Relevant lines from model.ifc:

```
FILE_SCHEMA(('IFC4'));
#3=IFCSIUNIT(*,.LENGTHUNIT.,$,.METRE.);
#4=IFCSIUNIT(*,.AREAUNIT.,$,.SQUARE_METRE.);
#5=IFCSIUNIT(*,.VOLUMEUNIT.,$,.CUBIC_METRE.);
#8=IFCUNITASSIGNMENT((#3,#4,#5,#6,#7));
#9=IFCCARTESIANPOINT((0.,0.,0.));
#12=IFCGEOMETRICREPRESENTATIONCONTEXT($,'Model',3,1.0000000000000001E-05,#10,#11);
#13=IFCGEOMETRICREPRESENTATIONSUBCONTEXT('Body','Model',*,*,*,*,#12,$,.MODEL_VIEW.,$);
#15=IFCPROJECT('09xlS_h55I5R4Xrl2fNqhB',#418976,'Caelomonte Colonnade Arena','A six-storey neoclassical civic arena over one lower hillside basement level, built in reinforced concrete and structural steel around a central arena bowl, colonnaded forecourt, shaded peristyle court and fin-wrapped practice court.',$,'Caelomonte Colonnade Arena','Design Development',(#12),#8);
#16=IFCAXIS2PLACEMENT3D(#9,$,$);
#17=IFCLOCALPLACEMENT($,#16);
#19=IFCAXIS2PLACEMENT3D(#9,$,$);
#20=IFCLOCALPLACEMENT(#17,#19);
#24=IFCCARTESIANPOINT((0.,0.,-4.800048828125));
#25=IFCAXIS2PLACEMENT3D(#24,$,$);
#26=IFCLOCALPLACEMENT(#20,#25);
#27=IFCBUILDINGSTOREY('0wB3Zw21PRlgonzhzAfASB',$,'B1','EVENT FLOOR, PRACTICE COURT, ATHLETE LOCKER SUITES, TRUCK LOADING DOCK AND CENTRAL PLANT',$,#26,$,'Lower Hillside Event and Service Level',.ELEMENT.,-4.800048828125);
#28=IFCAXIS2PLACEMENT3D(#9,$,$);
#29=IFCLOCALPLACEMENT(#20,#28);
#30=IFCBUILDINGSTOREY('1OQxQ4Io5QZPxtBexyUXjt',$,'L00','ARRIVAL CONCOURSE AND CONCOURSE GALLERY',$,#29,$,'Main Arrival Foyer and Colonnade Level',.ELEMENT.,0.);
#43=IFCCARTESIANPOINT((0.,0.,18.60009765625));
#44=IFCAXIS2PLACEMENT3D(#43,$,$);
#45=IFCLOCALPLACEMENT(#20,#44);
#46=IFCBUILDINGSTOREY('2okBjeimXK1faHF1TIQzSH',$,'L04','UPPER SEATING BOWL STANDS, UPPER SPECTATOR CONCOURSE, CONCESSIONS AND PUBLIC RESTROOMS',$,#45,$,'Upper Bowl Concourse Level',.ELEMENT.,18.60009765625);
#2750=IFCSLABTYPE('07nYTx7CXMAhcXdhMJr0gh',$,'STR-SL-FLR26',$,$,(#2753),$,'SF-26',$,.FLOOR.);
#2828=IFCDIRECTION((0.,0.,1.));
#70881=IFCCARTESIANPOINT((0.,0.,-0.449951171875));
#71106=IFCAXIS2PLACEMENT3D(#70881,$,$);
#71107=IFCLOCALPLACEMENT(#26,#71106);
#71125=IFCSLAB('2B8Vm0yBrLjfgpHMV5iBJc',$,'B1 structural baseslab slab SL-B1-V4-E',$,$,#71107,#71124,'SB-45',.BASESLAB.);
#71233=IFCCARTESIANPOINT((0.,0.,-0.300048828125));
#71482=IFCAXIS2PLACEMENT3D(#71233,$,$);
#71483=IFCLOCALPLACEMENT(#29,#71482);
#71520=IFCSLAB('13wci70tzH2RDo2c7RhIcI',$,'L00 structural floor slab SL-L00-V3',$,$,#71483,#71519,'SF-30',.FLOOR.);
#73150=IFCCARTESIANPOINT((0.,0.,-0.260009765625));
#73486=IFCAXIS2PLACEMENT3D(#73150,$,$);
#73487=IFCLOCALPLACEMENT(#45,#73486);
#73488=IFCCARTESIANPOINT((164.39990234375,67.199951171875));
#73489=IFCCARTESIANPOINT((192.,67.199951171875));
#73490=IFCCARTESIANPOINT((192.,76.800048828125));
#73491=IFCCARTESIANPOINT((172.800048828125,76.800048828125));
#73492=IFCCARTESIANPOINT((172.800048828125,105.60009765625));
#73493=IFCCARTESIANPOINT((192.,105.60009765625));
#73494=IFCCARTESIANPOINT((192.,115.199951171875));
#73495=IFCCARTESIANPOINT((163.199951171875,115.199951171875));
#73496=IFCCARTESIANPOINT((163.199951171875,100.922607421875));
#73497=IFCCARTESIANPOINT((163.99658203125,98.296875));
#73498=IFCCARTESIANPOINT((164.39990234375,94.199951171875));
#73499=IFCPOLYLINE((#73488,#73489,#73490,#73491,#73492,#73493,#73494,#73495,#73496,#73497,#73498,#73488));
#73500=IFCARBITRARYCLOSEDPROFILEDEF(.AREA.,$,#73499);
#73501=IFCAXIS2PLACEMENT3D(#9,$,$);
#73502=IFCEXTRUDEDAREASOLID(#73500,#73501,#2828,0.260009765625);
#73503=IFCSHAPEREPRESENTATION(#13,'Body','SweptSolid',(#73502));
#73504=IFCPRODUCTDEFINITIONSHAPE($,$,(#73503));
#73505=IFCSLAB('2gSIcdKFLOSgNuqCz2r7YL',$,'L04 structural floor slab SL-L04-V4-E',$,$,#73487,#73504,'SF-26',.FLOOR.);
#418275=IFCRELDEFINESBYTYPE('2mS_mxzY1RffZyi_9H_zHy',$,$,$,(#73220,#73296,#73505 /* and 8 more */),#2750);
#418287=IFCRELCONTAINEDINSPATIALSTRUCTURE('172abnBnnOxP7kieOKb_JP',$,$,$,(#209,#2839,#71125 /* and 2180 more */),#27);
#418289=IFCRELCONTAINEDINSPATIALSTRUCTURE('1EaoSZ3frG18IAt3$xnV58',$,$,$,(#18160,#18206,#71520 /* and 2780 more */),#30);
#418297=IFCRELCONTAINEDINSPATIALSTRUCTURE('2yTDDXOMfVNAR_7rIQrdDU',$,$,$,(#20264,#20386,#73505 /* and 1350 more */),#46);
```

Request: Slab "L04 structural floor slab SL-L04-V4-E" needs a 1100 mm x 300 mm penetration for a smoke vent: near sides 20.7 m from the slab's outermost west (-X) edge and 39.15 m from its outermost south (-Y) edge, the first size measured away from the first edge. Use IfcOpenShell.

```python
import numpy as np
import ifcopenshell
import ifcopenshell.api.feature
import ifcopenshell.api.geometry
import ifcopenshell.api.root
import ifcopenshell.geom
import ifcopenshell.util.placement
import ifcopenshell.util.representation
import ifcopenshell.util.shape
import ifcopenshell.util.unit

model = ifcopenshell.open("model.ifc")
unit_scale = ifcopenshell.util.unit.calculate_unit_scale(model)
settings = ifcopenshell.geom.settings()


def volume(element):
    """Net volume in cubic metres, openings subtracted."""
    shape = ifcopenshell.geom.create_shape(settings, element)
    return ifcopenshell.util.shape.get_volume(shape.geometry)


slab = model.by_id(73505)
before = volume(slab)

# Extent in the slab's own axes, in metres. The edges named are its -X and -Y sides.
slab_shape = ifcopenshell.geom.create_shape(settings, slab)
vertices = ifcopenshell.util.shape.get_vertices(slab_shape.geometry)
x_min, y_min, bottom = vertices.min(axis=0)
top = vertices[:, 2].max()

opening = ifcopenshell.api.root.create_entity(model, ifc_class="IfcOpeningElement", name="Smoke vent opening", predefined_type="OPENING")
context = ifcopenshell.util.representation.get_context(model, "Model", "Body", "MODEL_VIEW")
width, depth = 1.1, 0.3
outline = [(0.0, 0.0), (width, 0.0), (width, depth), (0.0, depth), (0.0, 0.0)]
# Overshoot both faces by 50 mm so the cut is clean.
shape = ifcopenshell.api.geometry.add_slab_representation(
    model, context=context, depth=top - bottom + 0.1, polyline=outline
)
ifcopenshell.api.geometry.assign_representation(model, product=opening, representation=shape)

matrix = ifcopenshell.util.placement.get_local_placement(slab.ObjectPlacement)
matrix[:, 3] = matrix @ np.append(np.array([x_min + 20.7, y_min + 39.15, bottom - 0.05]) / unit_scale, 1.0)
ifcopenshell.api.geometry.edit_object_placement(model, product=opening, matrix=matrix, is_si=False)
ifcopenshell.api.feature.add_feature(model, feature=opening, element=slab)

after = volume(slab)

print(f"slab volume {before:.3f} -> {after:.3f} m3")

model.write("model_edited.ifc")
```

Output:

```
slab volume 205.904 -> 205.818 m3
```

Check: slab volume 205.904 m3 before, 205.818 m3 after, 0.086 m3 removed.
